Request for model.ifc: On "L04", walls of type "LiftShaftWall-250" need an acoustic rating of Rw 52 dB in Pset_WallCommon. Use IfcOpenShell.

First a look at what the model holds.

```python
import ifcopenshell
import ifcopenshell.util.element

model = ifcopenshell.open("model.ifc")
print(model.schema)
storey = next(s for s in model.by_type("IfcBuildingStorey") if s.Name == "L04")
walls = [e for e in ifcopenshell.util.element.get_decomposition(storey) if e.is_a("IfcWall")]
seen = {}
for e in walls:
    element_type = ifcopenshell.util.element.get_type(e)
    key = (element_type.Name if element_type != e and element_type else None, ifcopenshell.util.element.get_pset(e, "Pset_WallCommon", "AcousticRating"))
    seen[key] = seen.get(key, 0) + 1
for (name, value), count in sorted(seen.items(), key=str):
    print(count, "x", name, "|", value)
```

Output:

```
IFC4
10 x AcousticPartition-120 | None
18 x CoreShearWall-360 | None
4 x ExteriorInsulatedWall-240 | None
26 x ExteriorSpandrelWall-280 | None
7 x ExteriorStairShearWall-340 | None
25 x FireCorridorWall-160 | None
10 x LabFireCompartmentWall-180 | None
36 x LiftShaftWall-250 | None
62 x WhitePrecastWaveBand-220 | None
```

```python
import ifcopenshell
import ifcopenshell.api.pset
import ifcopenshell.util.element

model = ifcopenshell.open("model.ifc")

storey = next(s for s in model.by_type("IfcBuildingStorey") if s.Name == "L04")
walls = [e for e in ifcopenshell.util.element.get_decomposition(storey) if e.is_a("IfcWall")]

count = 0
for e in walls:
    element_type = ifcopenshell.util.element.get_type(e)
    if element_type in (None, e) or element_type.Name != "LiftShaftWall-250":
        continue
    # add_pset returns the element's existing set when there is one.
    pset = ifcopenshell.api.pset.add_pset(model, product=e, name="Pset_WallCommon")
    ifcopenshell.api.pset.edit_pset(model, pset=pset, properties={"AcousticRating": "Rw 52 dB"})
    count += 1

print(count, "walls updated")

model.write("model-out.ifc")
```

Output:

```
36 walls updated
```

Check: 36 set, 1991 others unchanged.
